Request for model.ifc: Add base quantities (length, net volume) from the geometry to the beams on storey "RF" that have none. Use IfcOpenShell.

First a look at what the model holds.

```python
import ifcopenshell
import ifcopenshell.util.element
import ifcopenshell.util.unit

model = ifcopenshell.open("model.ifc")
print(model.schema)
for unit_type in ("LENGTHUNIT", "AREAUNIT", "VOLUMEUNIT"):
    print(unit_type, ifcopenshell.util.unit.calculate_unit_scale(model, unit_type))
storey = next(s for s in model.by_type("IfcBuildingStorey") if s.Name == "RF")
beams = [e for e in ifcopenshell.util.element.get_decomposition(storey) if e.is_a("IfcBeam")]
for e in sorted(beams, key=lambda e: e.id()):
    print(e.id(), e.is_a(), e.Name, list(ifcopenshell.util.element.get_psets(e, qtos_only=True)), sep=" | ")
```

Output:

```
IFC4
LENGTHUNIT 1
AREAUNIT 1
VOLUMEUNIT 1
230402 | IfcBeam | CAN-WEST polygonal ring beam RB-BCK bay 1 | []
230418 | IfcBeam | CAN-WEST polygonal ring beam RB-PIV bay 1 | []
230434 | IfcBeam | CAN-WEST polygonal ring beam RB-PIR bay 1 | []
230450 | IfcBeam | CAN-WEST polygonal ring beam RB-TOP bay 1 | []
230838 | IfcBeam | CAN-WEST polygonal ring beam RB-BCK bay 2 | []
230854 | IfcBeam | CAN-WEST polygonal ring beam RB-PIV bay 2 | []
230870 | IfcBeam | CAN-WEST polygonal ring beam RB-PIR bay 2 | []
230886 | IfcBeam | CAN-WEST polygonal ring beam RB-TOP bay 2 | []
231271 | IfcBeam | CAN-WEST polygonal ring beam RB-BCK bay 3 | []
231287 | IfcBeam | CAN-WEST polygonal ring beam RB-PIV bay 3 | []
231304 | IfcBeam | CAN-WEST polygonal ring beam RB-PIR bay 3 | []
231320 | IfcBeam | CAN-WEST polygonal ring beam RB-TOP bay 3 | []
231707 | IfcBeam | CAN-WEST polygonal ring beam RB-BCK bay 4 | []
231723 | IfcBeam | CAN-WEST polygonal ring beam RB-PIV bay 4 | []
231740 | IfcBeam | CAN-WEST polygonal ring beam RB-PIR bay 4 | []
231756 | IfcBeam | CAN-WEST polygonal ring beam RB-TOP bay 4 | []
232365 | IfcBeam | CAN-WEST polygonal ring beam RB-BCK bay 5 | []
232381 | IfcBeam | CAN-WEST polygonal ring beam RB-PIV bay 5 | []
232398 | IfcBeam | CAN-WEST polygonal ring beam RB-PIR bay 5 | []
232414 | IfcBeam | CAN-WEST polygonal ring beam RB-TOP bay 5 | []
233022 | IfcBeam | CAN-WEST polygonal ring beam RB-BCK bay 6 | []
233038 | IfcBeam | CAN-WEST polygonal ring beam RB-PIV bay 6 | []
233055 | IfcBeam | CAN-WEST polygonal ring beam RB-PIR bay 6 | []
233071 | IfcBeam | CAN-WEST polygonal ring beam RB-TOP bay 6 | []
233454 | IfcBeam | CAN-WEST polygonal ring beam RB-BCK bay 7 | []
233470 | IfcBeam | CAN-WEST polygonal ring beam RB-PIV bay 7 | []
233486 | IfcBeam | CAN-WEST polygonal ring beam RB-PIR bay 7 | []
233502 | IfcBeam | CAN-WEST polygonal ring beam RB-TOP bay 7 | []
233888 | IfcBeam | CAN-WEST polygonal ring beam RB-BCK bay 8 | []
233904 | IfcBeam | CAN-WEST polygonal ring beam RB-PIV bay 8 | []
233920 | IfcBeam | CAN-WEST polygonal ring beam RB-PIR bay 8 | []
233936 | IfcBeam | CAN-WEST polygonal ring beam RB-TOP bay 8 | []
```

```python
import ifcopenshell
import ifcopenshell.api.pset
import ifcopenshell.geom
import ifcopenshell.util.element
import ifcopenshell.util.shape
import ifcopenshell.util.unit

model = ifcopenshell.open("model.ifc")
unit_scale = ifcopenshell.util.unit.calculate_unit_scale(model)
volume_scale = ifcopenshell.util.unit.calculate_unit_scale(model, "VOLUMEUNIT")
settings = ifcopenshell.geom.settings()

storey = next(s for s in model.by_type("IfcBuildingStorey") if s.Name == "RF")
beams = [e for e in ifcopenshell.util.element.get_decomposition(storey) if e.is_a("IfcBeam")]

for e in sorted(beams, key=lambda e: e.id()):
    if ifcopenshell.util.element.get_psets(e, qtos_only=True, should_inherit=False):
        continue
    # Geometry comes back in metres, in the element's own axes.
    shape = ifcopenshell.geom.create_shape(settings, e)
    values = {
        "Length": ifcopenshell.util.shape.get_max_xyz(shape.geometry) / unit_scale,
        "NetVolume": ifcopenshell.util.shape.get_volume(shape.geometry) / volume_scale,
    }
    qto = ifcopenshell.api.pset.add_qto(model, product=e, name="Qto_BeamBaseQuantities")
    ifcopenshell.api.pset.edit_qto(model, qto=qto, properties=values)
    print(e.id(), {k: round(v, 3) for k, v in values.items()})

model.write("model_updated.ifc")
```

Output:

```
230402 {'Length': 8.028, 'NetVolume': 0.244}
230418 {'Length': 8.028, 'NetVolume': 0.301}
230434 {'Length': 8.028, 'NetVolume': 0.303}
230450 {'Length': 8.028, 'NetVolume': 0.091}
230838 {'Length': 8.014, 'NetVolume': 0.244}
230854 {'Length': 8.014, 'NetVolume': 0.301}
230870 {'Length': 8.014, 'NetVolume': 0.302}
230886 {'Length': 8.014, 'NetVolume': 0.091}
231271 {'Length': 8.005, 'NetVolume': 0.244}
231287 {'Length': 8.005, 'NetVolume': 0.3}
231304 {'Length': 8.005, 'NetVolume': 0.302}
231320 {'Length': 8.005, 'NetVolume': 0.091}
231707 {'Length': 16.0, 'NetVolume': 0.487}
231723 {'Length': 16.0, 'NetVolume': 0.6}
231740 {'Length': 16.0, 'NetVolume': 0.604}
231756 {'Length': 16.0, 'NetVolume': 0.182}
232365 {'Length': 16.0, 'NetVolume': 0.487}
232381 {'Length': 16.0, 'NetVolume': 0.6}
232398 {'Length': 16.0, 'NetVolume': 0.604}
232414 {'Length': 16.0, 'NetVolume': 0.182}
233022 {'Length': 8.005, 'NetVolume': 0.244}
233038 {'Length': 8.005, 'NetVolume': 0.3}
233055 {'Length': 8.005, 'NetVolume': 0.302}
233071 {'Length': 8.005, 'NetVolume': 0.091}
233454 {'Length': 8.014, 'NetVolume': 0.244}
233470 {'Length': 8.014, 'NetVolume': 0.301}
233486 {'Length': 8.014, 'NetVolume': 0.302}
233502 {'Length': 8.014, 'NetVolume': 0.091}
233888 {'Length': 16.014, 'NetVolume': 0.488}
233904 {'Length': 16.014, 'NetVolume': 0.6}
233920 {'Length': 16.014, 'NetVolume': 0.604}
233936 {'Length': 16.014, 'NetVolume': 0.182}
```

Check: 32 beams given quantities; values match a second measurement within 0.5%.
